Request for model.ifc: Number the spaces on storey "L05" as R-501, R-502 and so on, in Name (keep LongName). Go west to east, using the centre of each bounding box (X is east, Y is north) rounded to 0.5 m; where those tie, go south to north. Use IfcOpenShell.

First a look at what the model holds.

```python
import ifcopenshell
import ifcopenshell.util.element
import ifcopenshell.util.placement

model = ifcopenshell.open("model.ifc")
print(model.schema)
storey = next(s for s in model.by_type("IfcBuildingStorey") if s.Name == "L05")
spaces = [e for e in ifcopenshell.util.element.get_decomposition(storey) if e.is_a("IfcSpace")]
for e in sorted(spaces, key=lambda e: e.id()):
    origin = ifcopenshell.util.placement.get_local_placement(e.ObjectPlacement)[:3, 3]
    print(e.id(), e.Name, e.LongName, origin.round(2) + 0.0, sep=" | ")
```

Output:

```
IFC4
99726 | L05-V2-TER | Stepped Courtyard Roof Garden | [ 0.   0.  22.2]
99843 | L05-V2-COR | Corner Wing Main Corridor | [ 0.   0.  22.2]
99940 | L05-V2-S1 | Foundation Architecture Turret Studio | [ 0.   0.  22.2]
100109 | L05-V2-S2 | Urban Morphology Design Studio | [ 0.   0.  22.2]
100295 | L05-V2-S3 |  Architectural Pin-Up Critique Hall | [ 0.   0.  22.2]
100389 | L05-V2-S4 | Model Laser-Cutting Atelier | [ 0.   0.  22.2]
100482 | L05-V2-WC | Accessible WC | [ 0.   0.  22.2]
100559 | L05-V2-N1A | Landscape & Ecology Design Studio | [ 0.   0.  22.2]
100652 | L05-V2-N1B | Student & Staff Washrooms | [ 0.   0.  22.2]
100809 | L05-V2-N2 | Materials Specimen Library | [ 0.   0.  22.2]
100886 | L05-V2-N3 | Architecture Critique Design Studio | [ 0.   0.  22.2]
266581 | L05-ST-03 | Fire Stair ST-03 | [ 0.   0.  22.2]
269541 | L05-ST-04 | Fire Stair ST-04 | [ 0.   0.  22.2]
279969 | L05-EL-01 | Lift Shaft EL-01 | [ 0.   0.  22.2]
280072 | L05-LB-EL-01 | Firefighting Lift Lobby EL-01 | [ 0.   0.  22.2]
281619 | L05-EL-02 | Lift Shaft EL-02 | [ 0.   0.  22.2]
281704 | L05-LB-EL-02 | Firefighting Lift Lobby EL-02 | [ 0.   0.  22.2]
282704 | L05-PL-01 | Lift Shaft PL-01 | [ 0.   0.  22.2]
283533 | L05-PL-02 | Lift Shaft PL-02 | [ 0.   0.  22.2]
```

```python
import ifcopenshell
import ifcopenshell.geom
import ifcopenshell.util.element
import ifcopenshell.util.shape

model = ifcopenshell.open("model.ifc")
settings = ifcopenshell.geom.settings()
settings.set("use-world-coords", True)


def centre(element):
    shape = ifcopenshell.geom.create_shape(settings, element)
    return ifcopenshell.util.shape.get_bbox_centroid(shape.geometry)


storey = next(s for s in model.by_type("IfcBuildingStorey") if s.Name == "L05")
spaces = [e for e in ifcopenshell.util.element.get_decomposition(storey) if e.is_a("IfcSpace")]

# Insertion points can sit at a corner or the storey origin, so sort by the geometry (in metres).
centres = {e: centre(e) for e in spaces}
spaces.sort(key=lambda e: (round(centres[e][0] / 0.5), centres[e][1]))

for i, e in enumerate(spaces, start=1):
    number = f"R-5{i:02d}"
    e.Name = number
    print(e.id(), number)

model.write("model-out.ifc")
```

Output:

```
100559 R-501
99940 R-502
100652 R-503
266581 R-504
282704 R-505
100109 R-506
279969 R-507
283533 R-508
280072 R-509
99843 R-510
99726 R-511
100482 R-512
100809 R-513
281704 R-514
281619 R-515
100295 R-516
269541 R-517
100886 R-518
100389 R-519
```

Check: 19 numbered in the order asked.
